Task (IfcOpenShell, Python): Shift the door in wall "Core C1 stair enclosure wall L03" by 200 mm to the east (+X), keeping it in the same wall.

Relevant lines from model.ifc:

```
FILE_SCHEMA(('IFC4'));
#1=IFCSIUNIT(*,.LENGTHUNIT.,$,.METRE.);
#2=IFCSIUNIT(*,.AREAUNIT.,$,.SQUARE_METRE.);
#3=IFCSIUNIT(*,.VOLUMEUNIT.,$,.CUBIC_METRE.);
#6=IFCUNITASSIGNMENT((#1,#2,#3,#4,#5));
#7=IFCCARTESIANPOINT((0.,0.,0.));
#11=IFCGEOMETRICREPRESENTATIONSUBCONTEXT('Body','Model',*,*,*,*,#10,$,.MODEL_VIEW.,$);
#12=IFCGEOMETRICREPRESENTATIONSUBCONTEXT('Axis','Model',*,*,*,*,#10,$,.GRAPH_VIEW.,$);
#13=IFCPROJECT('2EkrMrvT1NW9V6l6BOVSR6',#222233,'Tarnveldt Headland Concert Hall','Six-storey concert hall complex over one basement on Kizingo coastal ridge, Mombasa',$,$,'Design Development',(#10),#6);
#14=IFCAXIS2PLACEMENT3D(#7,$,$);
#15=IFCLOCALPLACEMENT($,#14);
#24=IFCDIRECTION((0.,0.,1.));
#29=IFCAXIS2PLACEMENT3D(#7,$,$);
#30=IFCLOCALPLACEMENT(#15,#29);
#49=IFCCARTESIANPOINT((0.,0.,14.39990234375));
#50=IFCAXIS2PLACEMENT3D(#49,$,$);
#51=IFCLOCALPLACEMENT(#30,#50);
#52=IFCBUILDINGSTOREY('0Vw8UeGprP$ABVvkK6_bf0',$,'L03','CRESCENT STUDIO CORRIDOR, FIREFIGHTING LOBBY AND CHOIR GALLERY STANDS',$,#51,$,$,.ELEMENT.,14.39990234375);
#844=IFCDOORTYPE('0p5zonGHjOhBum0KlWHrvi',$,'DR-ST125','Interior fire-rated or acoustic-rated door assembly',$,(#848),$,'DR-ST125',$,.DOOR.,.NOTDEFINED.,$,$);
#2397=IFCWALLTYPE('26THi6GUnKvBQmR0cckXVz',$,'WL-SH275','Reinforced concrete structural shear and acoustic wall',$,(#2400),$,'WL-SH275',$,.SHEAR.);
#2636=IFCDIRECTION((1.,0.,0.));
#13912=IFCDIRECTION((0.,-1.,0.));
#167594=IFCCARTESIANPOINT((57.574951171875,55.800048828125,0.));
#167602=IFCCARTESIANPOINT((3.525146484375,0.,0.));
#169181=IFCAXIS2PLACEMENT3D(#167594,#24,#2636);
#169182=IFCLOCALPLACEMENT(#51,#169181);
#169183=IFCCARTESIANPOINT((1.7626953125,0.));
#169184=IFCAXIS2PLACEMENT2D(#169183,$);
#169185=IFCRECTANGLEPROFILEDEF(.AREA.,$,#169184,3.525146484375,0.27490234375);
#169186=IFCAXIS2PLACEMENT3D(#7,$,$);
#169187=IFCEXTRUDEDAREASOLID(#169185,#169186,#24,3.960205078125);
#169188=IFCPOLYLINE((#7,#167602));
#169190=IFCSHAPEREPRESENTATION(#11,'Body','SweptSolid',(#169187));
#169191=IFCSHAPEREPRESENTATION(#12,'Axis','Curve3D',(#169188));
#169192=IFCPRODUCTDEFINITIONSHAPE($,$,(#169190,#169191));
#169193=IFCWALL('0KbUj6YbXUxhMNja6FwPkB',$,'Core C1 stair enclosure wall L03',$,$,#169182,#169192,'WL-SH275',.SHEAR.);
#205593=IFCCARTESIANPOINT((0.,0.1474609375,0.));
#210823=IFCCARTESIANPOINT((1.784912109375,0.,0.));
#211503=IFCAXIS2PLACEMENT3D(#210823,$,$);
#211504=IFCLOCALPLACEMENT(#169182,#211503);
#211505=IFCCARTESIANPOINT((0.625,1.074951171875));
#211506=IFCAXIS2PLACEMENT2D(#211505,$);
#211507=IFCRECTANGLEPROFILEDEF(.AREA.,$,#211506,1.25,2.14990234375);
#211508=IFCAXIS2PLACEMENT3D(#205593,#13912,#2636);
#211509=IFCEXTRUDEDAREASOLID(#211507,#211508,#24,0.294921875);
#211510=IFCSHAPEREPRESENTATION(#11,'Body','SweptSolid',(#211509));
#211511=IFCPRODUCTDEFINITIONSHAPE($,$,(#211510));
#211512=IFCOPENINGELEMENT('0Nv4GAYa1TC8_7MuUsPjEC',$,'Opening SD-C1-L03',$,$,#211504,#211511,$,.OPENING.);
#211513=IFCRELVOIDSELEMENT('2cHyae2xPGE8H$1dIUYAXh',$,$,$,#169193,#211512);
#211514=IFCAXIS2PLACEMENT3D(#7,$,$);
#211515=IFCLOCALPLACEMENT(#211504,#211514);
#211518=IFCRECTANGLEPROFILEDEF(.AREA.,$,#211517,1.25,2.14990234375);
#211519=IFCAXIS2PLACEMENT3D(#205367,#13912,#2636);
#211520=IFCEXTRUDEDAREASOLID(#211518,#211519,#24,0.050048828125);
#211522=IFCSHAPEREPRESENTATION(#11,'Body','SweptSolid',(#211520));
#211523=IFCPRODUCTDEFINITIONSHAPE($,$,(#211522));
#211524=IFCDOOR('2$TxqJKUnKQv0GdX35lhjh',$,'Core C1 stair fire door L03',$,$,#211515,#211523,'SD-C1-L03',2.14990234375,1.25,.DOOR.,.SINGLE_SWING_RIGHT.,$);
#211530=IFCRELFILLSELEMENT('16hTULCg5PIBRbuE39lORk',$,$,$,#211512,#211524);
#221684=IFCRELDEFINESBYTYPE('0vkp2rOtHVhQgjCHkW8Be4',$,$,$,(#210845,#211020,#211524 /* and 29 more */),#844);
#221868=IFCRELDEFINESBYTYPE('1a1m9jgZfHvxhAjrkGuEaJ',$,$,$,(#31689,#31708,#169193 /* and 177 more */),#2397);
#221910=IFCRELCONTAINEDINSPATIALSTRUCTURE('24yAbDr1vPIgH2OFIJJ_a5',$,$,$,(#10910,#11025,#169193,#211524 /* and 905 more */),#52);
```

```python
import ifcopenshell
import ifcopenshell.api.geometry
import ifcopenshell.util.placement

model = ifcopenshell.open("model.ifc")

door = model.by_guid("2$TxqJKUnKQv0GdX35lhjh")
opening = door.FillsVoids[0].RelatingOpeningElement
wall = opening.VoidsElements[0].RelatingBuildingElement

wall_matrix = ifcopenshell.util.placement.get_local_placement(wall.ObjectPlacement)
shift = wall_matrix[:3, 0] * 0.2
before = ifcopenshell.util.placement.get_local_placement(door.ObjectPlacement)[:3, 3].copy()

# The door is placed relative to its opening, so it follows when the opening moves.
matrix = ifcopenshell.util.placement.get_local_placement(opening.ObjectPlacement)
matrix[:3, 3] += shift
ifcopenshell.api.geometry.edit_object_placement(
    model, product=opening, matrix=matrix, is_si=False, should_transform_children=True
)

after = ifcopenshell.util.placement.get_local_placement(door.ObjectPlacement)[:3, 3]
print("door moved by", (after - before).round(3) + 0.0)

model.write("model_v2.ifc")
```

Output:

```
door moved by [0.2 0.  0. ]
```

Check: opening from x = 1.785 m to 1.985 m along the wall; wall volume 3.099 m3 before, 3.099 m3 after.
